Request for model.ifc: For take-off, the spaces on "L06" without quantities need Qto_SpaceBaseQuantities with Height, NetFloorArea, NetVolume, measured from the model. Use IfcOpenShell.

First a look at what the model holds.

```python
import ifcopenshell
import ifcopenshell.util.element
import ifcopenshell.util.unit

model = ifcopenshell.open("model.ifc")
print(model.schema)
for unit_type in ("LENGTHUNIT", "AREAUNIT", "VOLUMEUNIT"):
    print(unit_type, ifcopenshell.util.unit.calculate_unit_scale(model, unit_type))
storey = next(s for s in model.by_type("IfcBuildingStorey") if s.Name == "L06")
spaces = [e for e in ifcopenshell.util.element.get_decomposition(storey) if e.is_a("IfcSpace")]
for e in sorted(spaces, key=lambda e: e.id()):
    print(e.id(), e.is_a(), e.Name, list(ifcopenshell.util.element.get_psets(e, qtos_only=True)), sep=" | ")
```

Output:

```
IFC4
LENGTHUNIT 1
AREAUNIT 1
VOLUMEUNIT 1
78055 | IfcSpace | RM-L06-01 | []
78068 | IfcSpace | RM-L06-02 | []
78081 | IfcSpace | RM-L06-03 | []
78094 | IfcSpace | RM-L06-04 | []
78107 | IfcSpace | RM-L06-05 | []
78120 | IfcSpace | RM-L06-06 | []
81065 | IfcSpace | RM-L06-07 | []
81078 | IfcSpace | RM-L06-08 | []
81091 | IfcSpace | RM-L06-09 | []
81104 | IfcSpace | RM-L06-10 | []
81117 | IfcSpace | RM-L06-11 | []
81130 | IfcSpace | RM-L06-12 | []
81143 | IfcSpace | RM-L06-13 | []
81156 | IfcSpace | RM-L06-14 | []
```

```python
import ifcopenshell
import ifcopenshell.api.pset
import ifcopenshell.geom
import ifcopenshell.util.element
import ifcopenshell.util.shape
import ifcopenshell.util.unit

model = ifcopenshell.open("model.ifc")
unit_scale = ifcopenshell.util.unit.calculate_unit_scale(model)
area_scale = ifcopenshell.util.unit.calculate_unit_scale(model, "AREAUNIT")
volume_scale = ifcopenshell.util.unit.calculate_unit_scale(model, "VOLUMEUNIT")
settings = ifcopenshell.geom.settings()

storey = next(s for s in model.by_type("IfcBuildingStorey") if s.Name == "L06")
spaces = [e for e in ifcopenshell.util.element.get_decomposition(storey) if e.is_a("IfcSpace")]

for e in sorted(spaces, key=lambda e: e.id()):
    if ifcopenshell.util.element.get_psets(e, qtos_only=True, should_inherit=False):
        continue
    # Geometry comes back in metres, in the element's own axes.
    shape = ifcopenshell.geom.create_shape(settings, e)
    values = {
        "Height": ifcopenshell.util.shape.get_z(shape.geometry) / unit_scale,
        "NetFloorArea": ifcopenshell.util.shape.get_footprint_area(shape.geometry) / area_scale,
        "NetVolume": ifcopenshell.util.shape.get_volume(shape.geometry) / volume_scale,
    }
    qto = ifcopenshell.api.pset.add_qto(model, product=e, name="Qto_SpaceBaseQuantities")
    ifcopenshell.api.pset.edit_qto(model, qto=qto, properties=values)
    print(e.id(), {k: round(v, 3) for k, v in values.items()})

model.write("model_updated.ifc")
```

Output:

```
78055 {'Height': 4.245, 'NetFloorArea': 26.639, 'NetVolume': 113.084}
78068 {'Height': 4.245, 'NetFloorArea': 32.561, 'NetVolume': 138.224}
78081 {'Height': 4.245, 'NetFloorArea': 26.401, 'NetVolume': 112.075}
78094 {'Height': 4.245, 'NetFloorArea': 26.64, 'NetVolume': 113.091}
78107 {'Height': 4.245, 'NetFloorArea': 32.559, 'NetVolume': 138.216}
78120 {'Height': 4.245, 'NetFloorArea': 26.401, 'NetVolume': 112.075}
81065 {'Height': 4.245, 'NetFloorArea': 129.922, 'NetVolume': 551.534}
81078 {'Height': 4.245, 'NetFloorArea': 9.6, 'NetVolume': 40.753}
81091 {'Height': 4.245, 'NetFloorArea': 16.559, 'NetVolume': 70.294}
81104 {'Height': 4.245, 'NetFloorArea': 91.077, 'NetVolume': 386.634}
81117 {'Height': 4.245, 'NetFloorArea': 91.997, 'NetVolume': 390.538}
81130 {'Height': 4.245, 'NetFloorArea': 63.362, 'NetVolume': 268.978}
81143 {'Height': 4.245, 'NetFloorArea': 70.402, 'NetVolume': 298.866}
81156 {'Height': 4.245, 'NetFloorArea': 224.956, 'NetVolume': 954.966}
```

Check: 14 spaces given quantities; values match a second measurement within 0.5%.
